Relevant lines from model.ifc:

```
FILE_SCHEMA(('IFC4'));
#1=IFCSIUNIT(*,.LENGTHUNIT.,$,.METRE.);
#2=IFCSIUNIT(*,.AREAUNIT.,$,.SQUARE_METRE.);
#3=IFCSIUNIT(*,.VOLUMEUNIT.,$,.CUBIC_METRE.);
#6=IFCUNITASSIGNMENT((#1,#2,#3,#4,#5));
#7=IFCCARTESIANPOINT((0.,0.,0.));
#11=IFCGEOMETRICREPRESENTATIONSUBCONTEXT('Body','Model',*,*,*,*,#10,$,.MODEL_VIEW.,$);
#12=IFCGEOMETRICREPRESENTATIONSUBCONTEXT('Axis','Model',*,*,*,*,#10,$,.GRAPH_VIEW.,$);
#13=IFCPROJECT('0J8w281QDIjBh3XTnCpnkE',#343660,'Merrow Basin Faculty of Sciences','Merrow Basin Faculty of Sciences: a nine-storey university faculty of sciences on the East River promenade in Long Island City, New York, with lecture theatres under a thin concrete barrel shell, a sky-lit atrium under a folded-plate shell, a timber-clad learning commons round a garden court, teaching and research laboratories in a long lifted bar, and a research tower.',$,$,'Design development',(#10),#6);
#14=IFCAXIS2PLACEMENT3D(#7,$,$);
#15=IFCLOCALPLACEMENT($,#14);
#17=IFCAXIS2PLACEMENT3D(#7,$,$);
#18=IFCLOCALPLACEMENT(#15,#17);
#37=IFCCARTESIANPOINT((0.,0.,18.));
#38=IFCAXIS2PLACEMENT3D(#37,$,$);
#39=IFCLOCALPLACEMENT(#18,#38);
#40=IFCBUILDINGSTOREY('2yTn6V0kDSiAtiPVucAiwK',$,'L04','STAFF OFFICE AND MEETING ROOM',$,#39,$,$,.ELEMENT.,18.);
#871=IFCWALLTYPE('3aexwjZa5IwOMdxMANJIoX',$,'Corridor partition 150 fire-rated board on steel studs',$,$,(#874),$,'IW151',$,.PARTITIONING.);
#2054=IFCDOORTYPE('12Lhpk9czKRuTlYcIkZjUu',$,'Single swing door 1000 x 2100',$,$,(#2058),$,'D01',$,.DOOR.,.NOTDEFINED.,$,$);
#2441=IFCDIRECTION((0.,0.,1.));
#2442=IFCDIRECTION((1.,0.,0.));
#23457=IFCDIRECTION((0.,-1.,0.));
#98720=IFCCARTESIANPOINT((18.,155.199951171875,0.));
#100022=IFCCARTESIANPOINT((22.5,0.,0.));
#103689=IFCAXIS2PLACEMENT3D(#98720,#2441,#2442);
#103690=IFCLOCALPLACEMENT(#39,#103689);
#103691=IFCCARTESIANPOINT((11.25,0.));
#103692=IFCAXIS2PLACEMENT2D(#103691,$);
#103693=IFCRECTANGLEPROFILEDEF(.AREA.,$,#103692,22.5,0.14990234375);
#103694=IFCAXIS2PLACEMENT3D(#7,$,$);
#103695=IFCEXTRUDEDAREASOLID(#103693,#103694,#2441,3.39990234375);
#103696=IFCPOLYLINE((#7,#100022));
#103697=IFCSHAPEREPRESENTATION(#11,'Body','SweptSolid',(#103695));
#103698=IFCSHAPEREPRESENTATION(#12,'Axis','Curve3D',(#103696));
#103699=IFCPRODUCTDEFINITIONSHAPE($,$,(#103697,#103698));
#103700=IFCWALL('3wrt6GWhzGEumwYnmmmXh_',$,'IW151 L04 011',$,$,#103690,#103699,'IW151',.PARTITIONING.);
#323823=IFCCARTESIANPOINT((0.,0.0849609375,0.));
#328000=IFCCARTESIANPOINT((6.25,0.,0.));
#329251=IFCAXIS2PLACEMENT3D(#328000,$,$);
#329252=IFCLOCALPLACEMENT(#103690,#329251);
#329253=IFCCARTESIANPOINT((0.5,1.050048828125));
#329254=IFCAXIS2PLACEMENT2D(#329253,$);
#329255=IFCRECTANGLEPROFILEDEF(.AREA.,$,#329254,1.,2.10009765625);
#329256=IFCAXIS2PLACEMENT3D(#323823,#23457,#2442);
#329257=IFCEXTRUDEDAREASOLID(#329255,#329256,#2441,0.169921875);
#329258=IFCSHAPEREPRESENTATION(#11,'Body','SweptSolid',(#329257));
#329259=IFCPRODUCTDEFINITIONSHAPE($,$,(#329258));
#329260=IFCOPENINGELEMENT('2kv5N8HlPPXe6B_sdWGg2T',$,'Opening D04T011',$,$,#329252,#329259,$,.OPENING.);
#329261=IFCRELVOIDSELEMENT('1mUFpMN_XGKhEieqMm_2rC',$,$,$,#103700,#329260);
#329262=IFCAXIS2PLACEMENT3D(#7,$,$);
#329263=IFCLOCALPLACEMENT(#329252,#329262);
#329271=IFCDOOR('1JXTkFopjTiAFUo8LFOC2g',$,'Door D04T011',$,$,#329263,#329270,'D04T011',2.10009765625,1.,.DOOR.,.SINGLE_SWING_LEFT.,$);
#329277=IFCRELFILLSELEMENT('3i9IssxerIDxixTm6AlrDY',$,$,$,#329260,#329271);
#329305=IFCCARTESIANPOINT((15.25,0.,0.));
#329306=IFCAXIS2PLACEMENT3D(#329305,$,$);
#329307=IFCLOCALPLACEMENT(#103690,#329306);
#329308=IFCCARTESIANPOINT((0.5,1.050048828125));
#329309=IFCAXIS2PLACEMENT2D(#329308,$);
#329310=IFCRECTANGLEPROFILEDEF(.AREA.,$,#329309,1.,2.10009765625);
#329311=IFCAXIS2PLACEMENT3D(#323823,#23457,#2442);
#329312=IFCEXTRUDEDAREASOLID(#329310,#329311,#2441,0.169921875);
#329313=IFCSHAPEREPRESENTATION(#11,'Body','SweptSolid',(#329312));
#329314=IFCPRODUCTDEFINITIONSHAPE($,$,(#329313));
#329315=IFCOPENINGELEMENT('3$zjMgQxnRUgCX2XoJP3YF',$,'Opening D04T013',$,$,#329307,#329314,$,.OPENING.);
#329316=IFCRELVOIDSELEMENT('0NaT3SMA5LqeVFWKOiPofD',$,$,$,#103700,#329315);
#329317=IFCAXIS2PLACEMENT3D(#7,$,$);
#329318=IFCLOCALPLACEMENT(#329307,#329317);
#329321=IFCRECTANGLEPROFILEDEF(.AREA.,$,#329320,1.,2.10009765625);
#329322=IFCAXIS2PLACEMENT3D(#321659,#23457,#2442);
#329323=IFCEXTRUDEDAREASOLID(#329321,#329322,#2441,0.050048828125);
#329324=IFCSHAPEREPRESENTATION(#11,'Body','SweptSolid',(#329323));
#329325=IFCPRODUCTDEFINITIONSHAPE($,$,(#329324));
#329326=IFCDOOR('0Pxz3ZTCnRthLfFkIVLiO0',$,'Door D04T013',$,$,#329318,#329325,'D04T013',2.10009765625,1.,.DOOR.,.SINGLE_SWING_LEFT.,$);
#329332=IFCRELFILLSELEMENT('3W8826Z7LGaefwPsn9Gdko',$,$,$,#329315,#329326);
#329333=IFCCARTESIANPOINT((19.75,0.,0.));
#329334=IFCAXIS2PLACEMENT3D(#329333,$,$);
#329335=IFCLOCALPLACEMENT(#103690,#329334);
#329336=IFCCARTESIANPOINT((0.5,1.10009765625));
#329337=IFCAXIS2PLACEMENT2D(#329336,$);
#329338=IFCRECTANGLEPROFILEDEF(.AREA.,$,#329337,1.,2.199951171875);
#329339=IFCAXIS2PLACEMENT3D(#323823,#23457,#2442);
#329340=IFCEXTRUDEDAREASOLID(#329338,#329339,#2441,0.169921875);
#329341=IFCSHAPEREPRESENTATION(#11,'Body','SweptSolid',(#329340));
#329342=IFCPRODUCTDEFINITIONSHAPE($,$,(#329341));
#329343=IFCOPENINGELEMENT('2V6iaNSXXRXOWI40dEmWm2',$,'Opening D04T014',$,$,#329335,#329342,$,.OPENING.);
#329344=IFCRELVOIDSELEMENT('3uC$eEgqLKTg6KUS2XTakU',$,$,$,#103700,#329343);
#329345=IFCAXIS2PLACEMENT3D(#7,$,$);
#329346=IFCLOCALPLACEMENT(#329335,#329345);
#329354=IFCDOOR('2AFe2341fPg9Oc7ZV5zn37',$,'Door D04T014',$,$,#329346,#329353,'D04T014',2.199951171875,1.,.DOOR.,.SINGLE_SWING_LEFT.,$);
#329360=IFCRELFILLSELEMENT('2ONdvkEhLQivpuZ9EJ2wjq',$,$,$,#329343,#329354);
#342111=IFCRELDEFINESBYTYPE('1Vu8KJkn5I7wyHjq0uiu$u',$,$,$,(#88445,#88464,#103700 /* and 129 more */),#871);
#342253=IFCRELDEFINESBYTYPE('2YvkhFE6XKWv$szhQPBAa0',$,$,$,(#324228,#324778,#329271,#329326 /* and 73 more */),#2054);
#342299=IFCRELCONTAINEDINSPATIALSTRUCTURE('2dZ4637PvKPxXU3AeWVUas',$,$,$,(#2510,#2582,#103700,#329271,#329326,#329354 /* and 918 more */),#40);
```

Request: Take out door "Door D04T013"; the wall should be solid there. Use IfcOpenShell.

```python
import ifcopenshell
import ifcopenshell.api.feature
import ifcopenshell.api.root
import ifcopenshell.geom
import ifcopenshell.util.shape

model = ifcopenshell.open("model.ifc")
settings = ifcopenshell.geom.settings()


def volume(element):
    """Net volume in cubic metres, openings subtracted."""
    shape = ifcopenshell.geom.create_shape(settings, element)
    return ifcopenshell.util.shape.get_volume(shape.geometry)


door = model.by_guid("0Pxz3ZTCnRthLfFkIVLiO0")
opening = door.FillsVoids[0].RelatingOpeningElement
wall = opening.VoidsElements[0].RelatingBuildingElement
before = volume(wall)

ifcopenshell.api.root.remove_product(model, product=door)
ifcopenshell.api.feature.remove_feature(model, feature=opening)

after = volume(wall)

print(f"wall volume {before:.3f} -> {after:.3f} m3")

model.write("model_updated.ifc")
```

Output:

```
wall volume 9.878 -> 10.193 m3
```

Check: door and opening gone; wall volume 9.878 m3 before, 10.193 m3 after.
